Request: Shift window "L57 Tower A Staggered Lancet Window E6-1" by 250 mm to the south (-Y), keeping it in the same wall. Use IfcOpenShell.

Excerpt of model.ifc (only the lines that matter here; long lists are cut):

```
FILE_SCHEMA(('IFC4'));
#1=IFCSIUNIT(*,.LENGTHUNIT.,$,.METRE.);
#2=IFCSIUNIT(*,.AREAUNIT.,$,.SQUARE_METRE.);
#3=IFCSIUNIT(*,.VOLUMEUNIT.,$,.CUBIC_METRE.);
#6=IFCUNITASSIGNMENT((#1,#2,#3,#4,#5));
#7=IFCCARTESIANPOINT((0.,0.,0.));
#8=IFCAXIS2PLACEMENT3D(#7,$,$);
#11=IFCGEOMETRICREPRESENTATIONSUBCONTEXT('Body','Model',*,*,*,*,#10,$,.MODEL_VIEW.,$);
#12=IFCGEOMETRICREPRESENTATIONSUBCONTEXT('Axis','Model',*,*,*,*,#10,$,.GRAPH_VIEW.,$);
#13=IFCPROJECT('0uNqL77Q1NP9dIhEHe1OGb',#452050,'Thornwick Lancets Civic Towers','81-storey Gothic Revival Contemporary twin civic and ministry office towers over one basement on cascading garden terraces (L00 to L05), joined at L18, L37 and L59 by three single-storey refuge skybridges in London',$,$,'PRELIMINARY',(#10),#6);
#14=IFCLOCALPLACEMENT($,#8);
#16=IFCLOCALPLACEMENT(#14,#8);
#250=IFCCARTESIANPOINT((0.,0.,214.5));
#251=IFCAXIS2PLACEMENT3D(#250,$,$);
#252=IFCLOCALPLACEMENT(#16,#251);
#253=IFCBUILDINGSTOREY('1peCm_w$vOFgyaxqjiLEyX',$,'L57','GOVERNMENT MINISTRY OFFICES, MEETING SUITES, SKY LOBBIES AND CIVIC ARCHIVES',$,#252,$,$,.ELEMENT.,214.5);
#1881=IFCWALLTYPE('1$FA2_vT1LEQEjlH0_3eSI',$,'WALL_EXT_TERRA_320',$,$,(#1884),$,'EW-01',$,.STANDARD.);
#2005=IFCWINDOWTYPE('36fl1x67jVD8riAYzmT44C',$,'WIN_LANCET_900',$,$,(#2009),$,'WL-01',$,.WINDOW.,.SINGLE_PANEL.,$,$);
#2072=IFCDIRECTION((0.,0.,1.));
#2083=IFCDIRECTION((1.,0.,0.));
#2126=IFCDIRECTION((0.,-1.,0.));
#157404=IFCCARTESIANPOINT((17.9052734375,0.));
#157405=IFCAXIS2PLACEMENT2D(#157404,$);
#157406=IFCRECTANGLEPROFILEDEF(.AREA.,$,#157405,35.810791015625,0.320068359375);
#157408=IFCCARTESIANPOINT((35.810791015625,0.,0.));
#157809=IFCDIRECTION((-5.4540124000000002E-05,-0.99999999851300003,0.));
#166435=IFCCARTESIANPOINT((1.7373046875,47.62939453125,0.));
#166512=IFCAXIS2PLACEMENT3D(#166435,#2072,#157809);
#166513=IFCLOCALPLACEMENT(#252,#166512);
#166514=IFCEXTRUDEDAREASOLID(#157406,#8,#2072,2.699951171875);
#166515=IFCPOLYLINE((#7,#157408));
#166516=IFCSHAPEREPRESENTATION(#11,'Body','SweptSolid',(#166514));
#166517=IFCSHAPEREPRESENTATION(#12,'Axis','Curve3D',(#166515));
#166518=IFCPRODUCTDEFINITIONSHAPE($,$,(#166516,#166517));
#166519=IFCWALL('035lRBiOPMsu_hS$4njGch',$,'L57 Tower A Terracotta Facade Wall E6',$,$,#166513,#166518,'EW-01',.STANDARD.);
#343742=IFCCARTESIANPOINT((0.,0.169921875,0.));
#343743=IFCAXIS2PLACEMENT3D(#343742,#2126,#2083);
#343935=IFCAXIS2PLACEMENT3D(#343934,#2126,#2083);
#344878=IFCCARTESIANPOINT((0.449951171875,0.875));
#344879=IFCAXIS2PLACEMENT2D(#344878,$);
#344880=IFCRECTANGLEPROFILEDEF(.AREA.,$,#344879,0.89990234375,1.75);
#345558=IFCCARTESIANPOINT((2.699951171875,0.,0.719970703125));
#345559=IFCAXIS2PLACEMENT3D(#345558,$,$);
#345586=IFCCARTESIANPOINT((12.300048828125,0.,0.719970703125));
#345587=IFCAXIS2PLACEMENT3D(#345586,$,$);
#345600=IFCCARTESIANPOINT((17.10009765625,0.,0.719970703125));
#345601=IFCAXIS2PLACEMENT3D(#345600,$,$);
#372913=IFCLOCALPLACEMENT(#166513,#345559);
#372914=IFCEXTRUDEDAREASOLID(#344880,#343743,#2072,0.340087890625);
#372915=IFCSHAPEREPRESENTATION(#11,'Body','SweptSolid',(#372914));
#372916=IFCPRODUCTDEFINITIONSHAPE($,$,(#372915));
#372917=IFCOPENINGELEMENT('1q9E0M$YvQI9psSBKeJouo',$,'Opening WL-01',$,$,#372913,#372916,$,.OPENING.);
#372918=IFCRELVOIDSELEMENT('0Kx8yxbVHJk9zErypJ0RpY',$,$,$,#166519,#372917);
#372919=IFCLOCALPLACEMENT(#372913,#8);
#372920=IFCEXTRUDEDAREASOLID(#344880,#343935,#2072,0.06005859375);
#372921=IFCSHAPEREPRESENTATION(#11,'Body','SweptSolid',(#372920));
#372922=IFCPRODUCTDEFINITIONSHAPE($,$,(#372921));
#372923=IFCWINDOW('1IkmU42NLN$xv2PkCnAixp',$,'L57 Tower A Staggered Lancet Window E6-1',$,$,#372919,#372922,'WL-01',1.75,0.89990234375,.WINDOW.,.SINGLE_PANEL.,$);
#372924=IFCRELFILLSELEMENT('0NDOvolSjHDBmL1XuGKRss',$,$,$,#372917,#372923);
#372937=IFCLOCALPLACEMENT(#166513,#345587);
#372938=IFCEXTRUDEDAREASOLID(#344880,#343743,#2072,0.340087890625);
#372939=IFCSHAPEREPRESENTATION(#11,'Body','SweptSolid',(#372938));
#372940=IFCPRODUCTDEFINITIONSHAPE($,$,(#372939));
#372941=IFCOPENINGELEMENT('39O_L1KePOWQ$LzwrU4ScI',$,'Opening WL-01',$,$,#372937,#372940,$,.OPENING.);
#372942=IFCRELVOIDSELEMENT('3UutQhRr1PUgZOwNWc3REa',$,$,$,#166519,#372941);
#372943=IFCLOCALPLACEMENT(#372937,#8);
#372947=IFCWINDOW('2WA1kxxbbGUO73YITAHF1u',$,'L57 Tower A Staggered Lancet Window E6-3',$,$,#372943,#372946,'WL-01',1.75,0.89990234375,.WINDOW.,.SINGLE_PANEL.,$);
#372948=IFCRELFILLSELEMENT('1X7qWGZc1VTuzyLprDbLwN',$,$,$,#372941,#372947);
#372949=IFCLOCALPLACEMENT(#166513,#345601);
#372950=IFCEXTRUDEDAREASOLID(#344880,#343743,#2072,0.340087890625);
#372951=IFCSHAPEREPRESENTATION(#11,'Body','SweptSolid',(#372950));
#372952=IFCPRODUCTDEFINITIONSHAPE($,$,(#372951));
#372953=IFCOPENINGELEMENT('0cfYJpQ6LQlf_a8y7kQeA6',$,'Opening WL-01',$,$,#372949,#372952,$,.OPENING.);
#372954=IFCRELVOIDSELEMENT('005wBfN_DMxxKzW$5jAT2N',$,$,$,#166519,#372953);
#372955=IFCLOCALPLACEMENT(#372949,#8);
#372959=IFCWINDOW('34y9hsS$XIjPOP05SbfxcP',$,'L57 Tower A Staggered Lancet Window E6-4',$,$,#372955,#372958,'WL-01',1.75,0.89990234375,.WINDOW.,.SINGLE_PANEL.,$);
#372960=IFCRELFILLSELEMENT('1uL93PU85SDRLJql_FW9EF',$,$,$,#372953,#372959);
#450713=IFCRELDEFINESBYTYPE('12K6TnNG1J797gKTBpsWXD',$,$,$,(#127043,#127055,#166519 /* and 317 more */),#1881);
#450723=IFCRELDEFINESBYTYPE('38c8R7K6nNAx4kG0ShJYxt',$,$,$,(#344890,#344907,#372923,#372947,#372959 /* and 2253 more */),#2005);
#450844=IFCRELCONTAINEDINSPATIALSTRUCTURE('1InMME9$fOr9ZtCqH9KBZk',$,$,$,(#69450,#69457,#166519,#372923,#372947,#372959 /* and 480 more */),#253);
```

```python
import ifcopenshell
import ifcopenshell.api.geometry
import ifcopenshell.util.placement

model = ifcopenshell.open("model.ifc")

window = model.by_id(372923)
opening = window.FillsVoids[0].RelatingOpeningElement
wall = opening.VoidsElements[0].RelatingBuildingElement

wall_matrix = ifcopenshell.util.placement.get_local_placement(wall.ObjectPlacement)
shift = wall_matrix[:3, 0] * 0.25
before = ifcopenshell.util.placement.get_local_placement(window.ObjectPlacement)[:3, 3].copy()

# The window is placed relative to its opening, so it follows when the opening moves.
matrix = ifcopenshell.util.placement.get_local_placement(opening.ObjectPlacement)
matrix[:3, 3] += shift
ifcopenshell.api.geometry.edit_object_placement(
    model, product=opening, matrix=matrix, is_si=False, should_transform_children=True
)

after = ifcopenshell.util.placement.get_local_placement(window.ObjectPlacement)[:3, 3]
print("window moved by", (after - before).round(3) + 0.0)

model.write("model_edited.ifc")
```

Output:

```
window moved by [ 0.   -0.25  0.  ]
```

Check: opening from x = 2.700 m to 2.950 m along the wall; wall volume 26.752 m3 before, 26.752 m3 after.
